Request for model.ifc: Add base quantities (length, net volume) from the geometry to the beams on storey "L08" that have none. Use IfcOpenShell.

First a look at what the model holds.

```python
import ifcopenshell
import ifcopenshell.util.element
import ifcopenshell.util.unit

model = ifcopenshell.open("model.ifc")
print(model.schema)
for unit_type in ("LENGTHUNIT", "AREAUNIT", "VOLUMEUNIT"):
    print(unit_type, ifcopenshell.util.unit.calculate_unit_scale(model, unit_type))
storey = next(s for s in model.by_type("IfcBuildingStorey") if s.Name == "L08")
beams = [e for e in ifcopenshell.util.element.get_decomposition(storey) if e.is_a("IfcBeam")]
for e in sorted(beams, key=lambda e: e.id()):
    print(e.id(), e.is_a(), e.Name, list(ifcopenshell.util.element.get_psets(e, qtos_only=True)), sep=" | ")
```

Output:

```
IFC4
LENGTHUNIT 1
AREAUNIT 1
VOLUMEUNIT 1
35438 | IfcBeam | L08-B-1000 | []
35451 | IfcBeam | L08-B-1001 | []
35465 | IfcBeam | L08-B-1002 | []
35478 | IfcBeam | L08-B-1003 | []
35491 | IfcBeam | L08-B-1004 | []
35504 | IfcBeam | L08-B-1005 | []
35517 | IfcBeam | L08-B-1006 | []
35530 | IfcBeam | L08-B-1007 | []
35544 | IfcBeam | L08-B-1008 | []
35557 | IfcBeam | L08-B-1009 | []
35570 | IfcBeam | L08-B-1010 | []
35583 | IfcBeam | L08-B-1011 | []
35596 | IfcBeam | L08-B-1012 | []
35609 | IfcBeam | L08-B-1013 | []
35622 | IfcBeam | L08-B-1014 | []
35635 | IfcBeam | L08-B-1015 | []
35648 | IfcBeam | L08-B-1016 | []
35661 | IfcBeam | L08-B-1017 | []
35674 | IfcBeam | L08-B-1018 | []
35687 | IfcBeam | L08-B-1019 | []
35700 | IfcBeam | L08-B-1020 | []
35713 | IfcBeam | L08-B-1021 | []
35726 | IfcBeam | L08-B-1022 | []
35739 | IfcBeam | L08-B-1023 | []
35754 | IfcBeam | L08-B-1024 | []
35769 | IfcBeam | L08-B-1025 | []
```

```python
import ifcopenshell
import ifcopenshell.api.pset
import ifcopenshell.geom
import ifcopenshell.util.element
import ifcopenshell.util.shape
import ifcopenshell.util.unit

model = ifcopenshell.open("model.ifc")
unit_scale = ifcopenshell.util.unit.calculate_unit_scale(model)
volume_scale = ifcopenshell.util.unit.calculate_unit_scale(model, "VOLUMEUNIT")
settings = ifcopenshell.geom.settings()

storey = next(s for s in model.by_type("IfcBuildingStorey") if s.Name == "L08")
beams = [e for e in ifcopenshell.util.element.get_decomposition(storey) if e.is_a("IfcBeam")]

for e in sorted(beams, key=lambda e: e.id()):
    if ifcopenshell.util.element.get_psets(e, qtos_only=True, should_inherit=False):
        continue
    # Geometry comes back in metres, in the element's own axes.
    shape = ifcopenshell.geom.create_shape(settings, e)
    values = {
        "Length": ifcopenshell.util.shape.get_max_xyz(shape.geometry) / unit_scale,
        "NetVolume": ifcopenshell.util.shape.get_volume(shape.geometry) / volume_scale,
    }
    qto = ifcopenshell.api.pset.add_qto(model, product=e, name="Qto_BeamBaseQuantities")
    ifcopenshell.api.pset.edit_qto(model, qto=qto, properties=values)
    print(e.id(), {k: round(v, 3) for k, v in values.items()})

model.write("model-out.ifc")
```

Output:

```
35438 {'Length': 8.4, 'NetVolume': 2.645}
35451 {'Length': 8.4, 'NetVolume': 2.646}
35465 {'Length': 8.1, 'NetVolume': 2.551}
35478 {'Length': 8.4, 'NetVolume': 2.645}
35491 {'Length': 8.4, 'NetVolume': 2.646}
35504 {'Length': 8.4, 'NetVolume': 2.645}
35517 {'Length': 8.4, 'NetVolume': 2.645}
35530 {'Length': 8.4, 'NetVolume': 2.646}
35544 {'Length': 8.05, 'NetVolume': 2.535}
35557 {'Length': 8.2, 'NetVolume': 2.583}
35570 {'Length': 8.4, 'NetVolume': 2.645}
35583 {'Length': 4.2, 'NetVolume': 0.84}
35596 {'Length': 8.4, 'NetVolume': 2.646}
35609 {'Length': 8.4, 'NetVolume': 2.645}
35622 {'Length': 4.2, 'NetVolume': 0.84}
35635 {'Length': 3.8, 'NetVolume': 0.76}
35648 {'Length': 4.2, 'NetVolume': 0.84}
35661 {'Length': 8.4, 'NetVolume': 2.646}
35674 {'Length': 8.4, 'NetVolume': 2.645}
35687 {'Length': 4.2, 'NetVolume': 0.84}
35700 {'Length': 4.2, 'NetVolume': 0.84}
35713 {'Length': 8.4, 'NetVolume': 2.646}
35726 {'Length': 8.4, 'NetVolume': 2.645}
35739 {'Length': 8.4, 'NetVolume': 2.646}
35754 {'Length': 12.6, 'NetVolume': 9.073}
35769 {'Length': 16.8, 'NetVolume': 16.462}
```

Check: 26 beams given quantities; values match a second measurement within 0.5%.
